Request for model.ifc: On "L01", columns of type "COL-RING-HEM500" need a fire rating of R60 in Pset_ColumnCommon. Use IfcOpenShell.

First a look at what the model holds.

```python
import ifcopenshell
import ifcopenshell.util.element

model = ifcopenshell.open("model.ifc")
print(model.schema)
storey = next(s for s in model.by_type("IfcBuildingStorey") if s.Name == "L01")
columns = [e for e in ifcopenshell.util.element.get_decomposition(storey) if e.is_a("IfcColumn")]
seen = {}
for e in columns:
    element_type = ifcopenshell.util.element.get_type(e)
    key = (element_type.Name if element_type != e and element_type else None, ifcopenshell.util.element.get_pset(e, "Pset_ColumnCommon", "FireRating"))
    seen[key] = seen.get(key, 0) + 1
for (name, value), count in sorted(seen.items(), key=str):
    print(count, "x", name, "|", value)
```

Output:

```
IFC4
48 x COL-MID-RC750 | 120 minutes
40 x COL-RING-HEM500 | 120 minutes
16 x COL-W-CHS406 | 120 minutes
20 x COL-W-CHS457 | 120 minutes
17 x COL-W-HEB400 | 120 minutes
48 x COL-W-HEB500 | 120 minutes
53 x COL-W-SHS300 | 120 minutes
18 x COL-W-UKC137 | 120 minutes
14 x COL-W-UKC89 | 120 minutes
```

```python
import ifcopenshell
import ifcopenshell.api.pset
import ifcopenshell.util.element

model = ifcopenshell.open("model.ifc")

storey = next(s for s in model.by_type("IfcBuildingStorey") if s.Name == "L01")
columns = [e for e in ifcopenshell.util.element.get_decomposition(storey) if e.is_a("IfcColumn")]

count = 0
for e in columns:
    element_type = ifcopenshell.util.element.get_type(e)
    if element_type in (None, e) or element_type.Name != "COL-RING-HEM500":
        continue
    # add_pset returns the element's existing set when there is one.
    pset = ifcopenshell.api.pset.add_pset(model, product=e, name="Pset_ColumnCommon")
    ifcopenshell.api.pset.edit_pset(model, pset=pset, properties={"FireRating": "R60"})
    count += 1

print(count, "columns updated")

model.write("model_updated.ifc")
```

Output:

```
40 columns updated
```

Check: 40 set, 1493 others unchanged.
